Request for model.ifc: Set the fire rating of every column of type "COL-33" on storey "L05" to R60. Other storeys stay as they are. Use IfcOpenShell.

First a look at what the model holds.

```python
import ifcopenshell
import ifcopenshell.util.element

model = ifcopenshell.open("model.ifc")
print(model.schema)
storey = next(s for s in model.by_type("IfcBuildingStorey") if s.Name == "L05")
columns = [e for e in ifcopenshell.util.element.get_decomposition(storey) if e.is_a("IfcColumn")]
seen = {}
for e in columns:
    element_type = ifcopenshell.util.element.get_type(e)
    key = (element_type.Name if element_type != e and element_type else None, ifcopenshell.util.element.get_pset(e, "Pset_ColumnCommon", "FireRating"))
    seen[key] = seen.get(key, 0) + 1
for (name, value), count in sorted(seen.items(), key=str):
    print(count, "x", name, "|", value)
```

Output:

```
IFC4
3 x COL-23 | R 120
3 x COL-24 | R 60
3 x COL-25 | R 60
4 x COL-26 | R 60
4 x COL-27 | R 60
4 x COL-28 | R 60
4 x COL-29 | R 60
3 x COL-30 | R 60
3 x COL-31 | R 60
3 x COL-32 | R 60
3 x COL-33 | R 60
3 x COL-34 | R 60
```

```python
import ifcopenshell
import ifcopenshell.api.pset
import ifcopenshell.util.element

model = ifcopenshell.open("model.ifc")

storey = next(s for s in model.by_type("IfcBuildingStorey") if s.Name == "L05")
columns = [e for e in ifcopenshell.util.element.get_decomposition(storey) if e.is_a("IfcColumn")]

count = 0
for e in columns:
    element_type = ifcopenshell.util.element.get_type(e)
    if element_type in (None, e) or element_type.Name != "COL-33":
        continue
    # add_pset returns the element's existing set when there is one.
    pset = ifcopenshell.api.pset.add_pset(model, product=e, name="Pset_ColumnCommon")
    ifcopenshell.api.pset.edit_pset(model, pset=pset, properties={"FireRating": "R60"})
    count += 1

print(count, "columns updated")

model.write("model_edited.ifc")
```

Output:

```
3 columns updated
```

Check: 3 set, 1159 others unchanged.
